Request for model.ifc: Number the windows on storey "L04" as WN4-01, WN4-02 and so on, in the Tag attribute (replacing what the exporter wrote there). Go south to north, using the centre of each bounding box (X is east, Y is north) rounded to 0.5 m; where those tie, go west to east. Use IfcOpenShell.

First a look at what the model holds.

```python
import ifcopenshell
import ifcopenshell.util.element
import ifcopenshell.util.placement

model = ifcopenshell.open("model.ifc")
print(model.schema)
storey = next(s for s in model.by_type("IfcBuildingStorey") if s.Name == "L04")
windows = [e for e in ifcopenshell.util.element.get_decomposition(storey) if e.is_a("IfcWindow")]
for e in sorted(windows, key=lambda e: e.id()):
    origin = ifcopenshell.util.placement.get_local_placement(e.ObjectPlacement)[:3, 3]
    print(e.id(), e.Tag, e.Name, origin.round(2) + 0.0, sep=" | ")
```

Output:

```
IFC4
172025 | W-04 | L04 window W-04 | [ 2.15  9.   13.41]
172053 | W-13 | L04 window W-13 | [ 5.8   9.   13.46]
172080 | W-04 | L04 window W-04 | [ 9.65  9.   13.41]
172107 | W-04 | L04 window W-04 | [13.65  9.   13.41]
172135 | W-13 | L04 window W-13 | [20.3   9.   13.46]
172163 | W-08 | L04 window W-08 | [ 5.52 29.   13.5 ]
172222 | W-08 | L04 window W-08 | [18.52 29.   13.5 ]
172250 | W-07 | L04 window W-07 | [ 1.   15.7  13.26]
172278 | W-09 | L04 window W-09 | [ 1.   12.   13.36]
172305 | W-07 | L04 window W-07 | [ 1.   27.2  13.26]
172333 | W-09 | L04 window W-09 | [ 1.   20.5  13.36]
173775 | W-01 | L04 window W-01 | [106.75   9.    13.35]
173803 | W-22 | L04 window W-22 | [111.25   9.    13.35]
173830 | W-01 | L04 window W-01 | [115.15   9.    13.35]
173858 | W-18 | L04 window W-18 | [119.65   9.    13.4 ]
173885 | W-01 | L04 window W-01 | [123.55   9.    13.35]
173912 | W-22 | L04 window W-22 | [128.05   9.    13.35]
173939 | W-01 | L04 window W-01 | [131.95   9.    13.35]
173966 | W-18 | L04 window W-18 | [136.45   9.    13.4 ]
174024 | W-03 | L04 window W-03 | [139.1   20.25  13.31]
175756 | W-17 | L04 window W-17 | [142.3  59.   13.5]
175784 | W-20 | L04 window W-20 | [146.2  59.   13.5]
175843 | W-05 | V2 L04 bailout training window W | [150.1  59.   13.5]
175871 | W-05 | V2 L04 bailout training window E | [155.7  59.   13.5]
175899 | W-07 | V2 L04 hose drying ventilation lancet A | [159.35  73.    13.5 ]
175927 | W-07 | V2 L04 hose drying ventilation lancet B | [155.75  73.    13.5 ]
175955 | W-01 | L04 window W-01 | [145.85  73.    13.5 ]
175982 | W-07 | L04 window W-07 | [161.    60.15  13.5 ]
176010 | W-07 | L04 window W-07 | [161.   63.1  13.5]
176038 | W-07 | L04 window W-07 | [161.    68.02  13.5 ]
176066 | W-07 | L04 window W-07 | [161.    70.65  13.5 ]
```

```python
import ifcopenshell
import ifcopenshell.geom
import ifcopenshell.util.element
import ifcopenshell.util.shape

model = ifcopenshell.open("model.ifc")
settings = ifcopenshell.geom.settings()
settings.set("use-world-coords", True)


def centre(element):
    shape = ifcopenshell.geom.create_shape(settings, element)
    return ifcopenshell.util.shape.get_bbox_centroid(shape.geometry)


storey = next(s for s in model.by_type("IfcBuildingStorey") if s.Name == "L04")
windows = [e for e in ifcopenshell.util.element.get_decomposition(storey) if e.is_a("IfcWindow")]

# Insertion points can sit at a corner or the storey origin, so sort by the geometry (in metres).
centres = {e: centre(e) for e in windows}
windows.sort(key=lambda e: (round(centres[e][1] / 0.5), centres[e][0]))

for i, e in enumerate(windows, start=1):
    number = f"WN4-{i:02d}"
    e.Tag = number
    print(e.id(), number)

model.write("model_rev.ifc")
```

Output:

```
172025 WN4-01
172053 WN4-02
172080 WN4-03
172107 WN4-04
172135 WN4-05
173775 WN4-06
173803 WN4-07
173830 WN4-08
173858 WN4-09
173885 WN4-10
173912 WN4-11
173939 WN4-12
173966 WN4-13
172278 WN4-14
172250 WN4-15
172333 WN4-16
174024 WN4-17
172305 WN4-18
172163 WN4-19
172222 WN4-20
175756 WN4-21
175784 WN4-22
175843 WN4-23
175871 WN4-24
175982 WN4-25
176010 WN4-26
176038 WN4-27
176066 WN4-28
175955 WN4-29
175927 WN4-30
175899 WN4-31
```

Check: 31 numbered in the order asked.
